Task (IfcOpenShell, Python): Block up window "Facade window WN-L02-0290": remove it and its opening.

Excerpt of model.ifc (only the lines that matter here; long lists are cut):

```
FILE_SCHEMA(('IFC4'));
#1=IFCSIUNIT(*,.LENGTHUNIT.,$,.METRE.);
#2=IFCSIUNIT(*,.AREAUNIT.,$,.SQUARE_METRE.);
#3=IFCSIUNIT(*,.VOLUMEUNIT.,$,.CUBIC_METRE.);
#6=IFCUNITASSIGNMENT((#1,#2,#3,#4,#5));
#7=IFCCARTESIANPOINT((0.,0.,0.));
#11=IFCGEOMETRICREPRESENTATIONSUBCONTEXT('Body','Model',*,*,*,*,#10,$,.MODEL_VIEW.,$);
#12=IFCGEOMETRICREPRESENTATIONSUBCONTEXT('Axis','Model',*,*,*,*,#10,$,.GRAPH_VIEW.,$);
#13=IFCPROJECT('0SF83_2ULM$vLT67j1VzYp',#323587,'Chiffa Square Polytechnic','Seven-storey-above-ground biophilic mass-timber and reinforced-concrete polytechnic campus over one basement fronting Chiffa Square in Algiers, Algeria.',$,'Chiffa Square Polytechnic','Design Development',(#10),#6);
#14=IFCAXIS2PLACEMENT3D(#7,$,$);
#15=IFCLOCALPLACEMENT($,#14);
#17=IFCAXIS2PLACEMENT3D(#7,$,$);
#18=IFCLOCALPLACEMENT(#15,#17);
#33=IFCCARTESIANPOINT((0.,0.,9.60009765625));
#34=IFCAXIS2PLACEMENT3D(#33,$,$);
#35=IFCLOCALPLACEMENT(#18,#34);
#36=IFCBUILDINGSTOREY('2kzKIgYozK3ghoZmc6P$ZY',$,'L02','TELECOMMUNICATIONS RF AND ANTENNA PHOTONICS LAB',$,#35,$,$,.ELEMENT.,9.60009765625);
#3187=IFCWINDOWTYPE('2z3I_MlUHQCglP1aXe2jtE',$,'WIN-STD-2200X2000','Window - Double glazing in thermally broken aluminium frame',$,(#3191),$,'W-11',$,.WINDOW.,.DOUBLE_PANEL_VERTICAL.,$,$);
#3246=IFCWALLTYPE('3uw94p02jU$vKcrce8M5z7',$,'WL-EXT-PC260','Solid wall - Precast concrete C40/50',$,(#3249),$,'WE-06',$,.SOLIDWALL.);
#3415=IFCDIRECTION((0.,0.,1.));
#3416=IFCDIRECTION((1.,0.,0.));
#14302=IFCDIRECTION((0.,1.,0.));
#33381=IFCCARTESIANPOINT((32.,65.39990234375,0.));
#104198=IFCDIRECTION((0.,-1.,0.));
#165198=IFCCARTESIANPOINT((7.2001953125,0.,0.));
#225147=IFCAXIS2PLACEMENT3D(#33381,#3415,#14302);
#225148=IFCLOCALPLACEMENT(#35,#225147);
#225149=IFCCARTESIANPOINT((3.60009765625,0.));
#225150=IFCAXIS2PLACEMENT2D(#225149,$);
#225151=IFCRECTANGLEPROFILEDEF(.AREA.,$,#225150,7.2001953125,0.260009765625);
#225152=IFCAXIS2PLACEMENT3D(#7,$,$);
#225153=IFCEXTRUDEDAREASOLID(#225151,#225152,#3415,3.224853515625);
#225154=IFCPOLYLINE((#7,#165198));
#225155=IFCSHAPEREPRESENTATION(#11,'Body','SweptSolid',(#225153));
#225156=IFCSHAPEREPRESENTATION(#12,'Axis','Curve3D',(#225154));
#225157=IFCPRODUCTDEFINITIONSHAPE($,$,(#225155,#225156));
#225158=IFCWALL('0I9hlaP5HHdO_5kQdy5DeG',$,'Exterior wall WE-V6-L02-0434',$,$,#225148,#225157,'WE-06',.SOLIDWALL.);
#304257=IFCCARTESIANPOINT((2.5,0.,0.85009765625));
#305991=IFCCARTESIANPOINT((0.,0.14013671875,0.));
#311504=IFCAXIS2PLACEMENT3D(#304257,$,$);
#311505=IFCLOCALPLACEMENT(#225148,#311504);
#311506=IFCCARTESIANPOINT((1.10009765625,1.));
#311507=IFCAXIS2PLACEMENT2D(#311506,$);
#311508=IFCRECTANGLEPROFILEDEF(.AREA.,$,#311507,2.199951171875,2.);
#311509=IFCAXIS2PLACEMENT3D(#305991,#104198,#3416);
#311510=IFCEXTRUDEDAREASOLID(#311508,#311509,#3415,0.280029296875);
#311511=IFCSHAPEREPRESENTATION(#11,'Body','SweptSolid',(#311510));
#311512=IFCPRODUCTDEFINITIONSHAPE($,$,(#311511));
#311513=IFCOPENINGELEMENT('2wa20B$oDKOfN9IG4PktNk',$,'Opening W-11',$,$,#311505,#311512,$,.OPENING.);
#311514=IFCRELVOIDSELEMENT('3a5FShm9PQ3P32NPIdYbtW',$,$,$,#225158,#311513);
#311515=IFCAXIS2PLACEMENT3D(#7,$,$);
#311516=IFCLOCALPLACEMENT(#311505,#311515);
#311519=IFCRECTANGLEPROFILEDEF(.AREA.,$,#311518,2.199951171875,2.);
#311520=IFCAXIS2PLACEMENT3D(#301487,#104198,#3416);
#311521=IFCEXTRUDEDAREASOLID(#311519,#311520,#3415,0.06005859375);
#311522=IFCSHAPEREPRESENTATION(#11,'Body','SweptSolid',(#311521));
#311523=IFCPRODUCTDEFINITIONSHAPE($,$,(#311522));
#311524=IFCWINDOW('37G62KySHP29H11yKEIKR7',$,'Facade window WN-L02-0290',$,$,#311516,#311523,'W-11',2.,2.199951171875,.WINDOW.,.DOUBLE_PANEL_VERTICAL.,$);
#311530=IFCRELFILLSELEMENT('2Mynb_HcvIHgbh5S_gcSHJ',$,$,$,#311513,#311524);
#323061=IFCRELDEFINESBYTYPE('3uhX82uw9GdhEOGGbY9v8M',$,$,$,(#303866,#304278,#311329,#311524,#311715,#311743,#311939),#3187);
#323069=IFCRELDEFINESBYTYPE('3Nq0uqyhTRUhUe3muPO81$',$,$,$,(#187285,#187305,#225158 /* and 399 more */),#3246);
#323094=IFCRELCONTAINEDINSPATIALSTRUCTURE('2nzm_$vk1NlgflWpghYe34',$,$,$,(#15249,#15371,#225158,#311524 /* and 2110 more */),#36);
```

```python
import ifcopenshell
import ifcopenshell.api.feature
import ifcopenshell.api.root
import ifcopenshell.geom
import ifcopenshell.util.shape

model = ifcopenshell.open("model.ifc")
settings = ifcopenshell.geom.settings()


def volume(element):
    """Net volume in cubic metres, openings subtracted."""
    shape = ifcopenshell.geom.create_shape(settings, element)
    return ifcopenshell.util.shape.get_volume(shape.geometry)


window = model.by_guid("37G62KySHP29H11yKEIKR7")
opening = window.FillsVoids[0].RelatingOpeningElement
wall = opening.VoidsElements[0].RelatingBuildingElement
before = volume(wall)

ifcopenshell.api.root.remove_product(model, product=window)
ifcopenshell.api.feature.remove_feature(model, feature=opening)

after = volume(wall)

print(f"wall volume {before:.3f} -> {after:.3f} m3")

model.write("model_edited.ifc")
```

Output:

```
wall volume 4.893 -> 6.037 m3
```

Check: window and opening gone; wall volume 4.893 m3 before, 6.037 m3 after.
